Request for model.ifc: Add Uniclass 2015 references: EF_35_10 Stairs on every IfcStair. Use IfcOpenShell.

First a look at what the model holds.

```python
import ifcopenshell

model = ifcopenshell.open("model.ifc")
print(model.schema)
print("classifications:", [c.Name for c in model.by_type("IfcClassification")])
for ifc_class in ("IfcDoor", "IfcRoof", "IfcStair", "IfcWall", "IfcWindow"):
    print(ifc_class, len(model.by_type(ifc_class)))
```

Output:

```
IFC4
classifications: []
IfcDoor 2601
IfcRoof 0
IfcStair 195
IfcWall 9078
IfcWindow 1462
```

```python
import ifcopenshell
import ifcopenshell.api.classification

model = ifcopenshell.open("model.ifc")

system = ifcopenshell.api.classification.add_classification(model, classification="Uniclass 2015")

codes = {
    "IfcStair": ("EF_35_10", "Stairs"),
}
for ifc_class, (code, name) in codes.items():
    products = model.by_type(ifc_class)
    ifcopenshell.api.classification.add_reference(
        model, products=products, classification=system, identification=code, name=name
    )
    print(code, len(products))

model.write("model-out.ifc")
```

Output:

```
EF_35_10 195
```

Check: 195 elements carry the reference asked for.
